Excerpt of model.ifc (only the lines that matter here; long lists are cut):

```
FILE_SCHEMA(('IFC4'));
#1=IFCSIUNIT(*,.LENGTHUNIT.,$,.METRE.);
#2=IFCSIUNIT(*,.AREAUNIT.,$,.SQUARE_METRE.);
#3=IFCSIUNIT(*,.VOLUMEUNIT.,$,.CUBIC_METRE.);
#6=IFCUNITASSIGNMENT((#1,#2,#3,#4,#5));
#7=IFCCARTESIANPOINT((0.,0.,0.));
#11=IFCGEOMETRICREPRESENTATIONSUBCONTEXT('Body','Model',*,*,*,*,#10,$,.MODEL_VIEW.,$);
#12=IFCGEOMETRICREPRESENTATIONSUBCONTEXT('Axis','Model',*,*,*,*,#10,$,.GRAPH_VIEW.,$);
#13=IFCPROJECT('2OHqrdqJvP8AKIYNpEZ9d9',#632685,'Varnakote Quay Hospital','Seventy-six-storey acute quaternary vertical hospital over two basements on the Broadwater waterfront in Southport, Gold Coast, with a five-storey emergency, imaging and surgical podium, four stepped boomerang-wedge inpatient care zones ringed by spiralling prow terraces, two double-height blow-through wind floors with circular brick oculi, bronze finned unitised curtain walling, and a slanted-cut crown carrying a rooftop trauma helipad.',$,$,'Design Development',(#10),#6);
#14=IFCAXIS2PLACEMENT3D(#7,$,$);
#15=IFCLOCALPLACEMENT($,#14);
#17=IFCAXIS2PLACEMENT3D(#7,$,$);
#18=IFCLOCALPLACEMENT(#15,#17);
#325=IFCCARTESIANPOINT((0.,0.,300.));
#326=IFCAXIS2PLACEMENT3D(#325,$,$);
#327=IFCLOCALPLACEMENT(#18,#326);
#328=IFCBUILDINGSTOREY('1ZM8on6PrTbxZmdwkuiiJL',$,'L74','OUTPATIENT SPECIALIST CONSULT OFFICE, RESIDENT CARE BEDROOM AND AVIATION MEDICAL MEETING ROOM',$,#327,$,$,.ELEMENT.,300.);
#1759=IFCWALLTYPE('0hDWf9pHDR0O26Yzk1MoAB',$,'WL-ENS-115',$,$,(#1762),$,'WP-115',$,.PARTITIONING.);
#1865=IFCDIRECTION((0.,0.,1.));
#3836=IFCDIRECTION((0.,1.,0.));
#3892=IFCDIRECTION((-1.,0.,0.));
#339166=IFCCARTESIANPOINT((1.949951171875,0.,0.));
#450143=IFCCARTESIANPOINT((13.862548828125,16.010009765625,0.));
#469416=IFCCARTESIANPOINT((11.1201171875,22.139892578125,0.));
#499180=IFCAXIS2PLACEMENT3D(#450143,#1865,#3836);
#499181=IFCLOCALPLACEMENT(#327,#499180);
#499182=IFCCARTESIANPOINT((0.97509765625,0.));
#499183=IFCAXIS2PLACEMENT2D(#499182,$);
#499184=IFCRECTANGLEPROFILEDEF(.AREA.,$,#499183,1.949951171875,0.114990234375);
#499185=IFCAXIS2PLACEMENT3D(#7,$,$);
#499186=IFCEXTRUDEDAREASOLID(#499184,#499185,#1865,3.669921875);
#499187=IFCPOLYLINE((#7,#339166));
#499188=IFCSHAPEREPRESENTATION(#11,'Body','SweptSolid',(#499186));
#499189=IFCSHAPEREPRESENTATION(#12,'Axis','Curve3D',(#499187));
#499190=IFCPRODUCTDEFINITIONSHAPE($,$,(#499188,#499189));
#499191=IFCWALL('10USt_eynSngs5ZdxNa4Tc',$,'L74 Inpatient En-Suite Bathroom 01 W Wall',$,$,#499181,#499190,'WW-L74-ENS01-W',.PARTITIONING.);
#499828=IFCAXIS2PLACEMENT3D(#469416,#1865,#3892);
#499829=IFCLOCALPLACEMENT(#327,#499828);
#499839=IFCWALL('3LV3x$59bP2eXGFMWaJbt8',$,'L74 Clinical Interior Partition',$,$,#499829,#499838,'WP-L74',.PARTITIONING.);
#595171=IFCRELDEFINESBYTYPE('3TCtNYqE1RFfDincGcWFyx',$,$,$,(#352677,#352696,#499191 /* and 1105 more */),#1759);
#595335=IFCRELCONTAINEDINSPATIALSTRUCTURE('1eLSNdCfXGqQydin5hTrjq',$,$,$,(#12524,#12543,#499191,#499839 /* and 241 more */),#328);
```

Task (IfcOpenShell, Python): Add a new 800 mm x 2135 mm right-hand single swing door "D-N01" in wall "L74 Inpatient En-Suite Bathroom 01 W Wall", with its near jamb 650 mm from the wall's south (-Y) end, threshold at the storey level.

```python
import numpy as np
import ifcopenshell
import ifcopenshell.api.feature
import ifcopenshell.api.geometry
import ifcopenshell.api.root
import ifcopenshell.api.spatial
import ifcopenshell.geom
import ifcopenshell.util.element
import ifcopenshell.util.placement
import ifcopenshell.util.representation
import ifcopenshell.util.shape
import ifcopenshell.util.unit

model = ifcopenshell.open("model.ifc")
unit_scale = ifcopenshell.util.unit.calculate_unit_scale(model)
settings = ifcopenshell.geom.settings()


def volume(element):
    """Net volume in cubic metres, openings subtracted."""
    shape = ifcopenshell.geom.create_shape(settings, element)
    return ifcopenshell.util.shape.get_volume(shape.geometry)


wall = model.by_guid("10USt_eynSngs5ZdxNa4Tc")
storey = ifcopenshell.util.element.get_container(wall, ifc_class="IfcBuildingStorey")
context = ifcopenshell.util.representation.get_context(model, "Model", "Body", "MODEL_VIEW")
before = volume(wall)

width, height, from_end, sill = 0.8, 2.135, 0.65, 0.0  # metres

# The wall runs along its own X axis, and the end named is its -X end.
wall_shape = ifcopenshell.geom.create_shape(settings, wall)
x, y, z = ifcopenshell.util.shape.get_vertices(wall_shape.geometry).T
start = x.min() + from_end
face, thickness = float(y.min()), float(y.max() - y.min())
wall_matrix = ifcopenshell.util.placement.get_local_placement(wall.ObjectPlacement)
level = ifcopenshell.util.placement.get_local_placement(storey.ObjectPlacement)[2, 3]


def in_wall(x, y):
    """Placement at x, y metres in the wall's axes, at sill height."""
    matrix = wall_matrix.copy()
    matrix[:, 3] = wall_matrix @ np.array([x / unit_scale, y / unit_scale, 0.0, 1.0])
    matrix[2, 3] = level + sill / unit_scale
    return matrix


# Opening: a box that overshoots both wall faces by 50 mm.
opening = ifcopenshell.api.root.create_entity(model, ifc_class="IfcOpeningElement", predefined_type="OPENING")
box = ifcopenshell.api.geometry.add_wall_representation(
    model, context=context, length=width, height=height, thickness=thickness + 0.1
)
ifcopenshell.api.geometry.assign_representation(model, product=opening, representation=box)
ifcopenshell.api.geometry.edit_object_placement(model, product=opening, matrix=in_wall(start, face - 0.05), is_si=False)
ifcopenshell.api.feature.add_feature(model, feature=opening, element=wall)

door = ifcopenshell.api.root.create_entity(model, ifc_class="IfcDoor", name="D-N01", predefined_type="DOOR")
door.OverallWidth, door.OverallHeight = width / unit_scale, height / unit_scale
door.OperationType = "SINGLE_SWING_RIGHT"
body = ifcopenshell.api.geometry.add_door_representation(
    model,
    context=context,
    overall_width=door.OverallWidth,
    overall_height=door.OverallHeight,
    operation_type="SINGLE_SWING_RIGHT",
    lining_properties={"LiningDepth": thickness / unit_scale, "ThresholdDepth": thickness / unit_scale},
)
ifcopenshell.api.geometry.assign_representation(model, product=door, representation=body)
ifcopenshell.api.spatial.assign_container(model, products=[door], relating_structure=storey)
ifcopenshell.api.feature.add_filling(model, opening=opening, element=door)

# The lining spans the wall, so the door starts at the wall face.
ifcopenshell.api.geometry.edit_object_placement(model, product=door, matrix=in_wall(start, face), is_si=False)

after = volume(wall)

print(f"wall volume {before:.3f} -> {after:.3f} m3")

model.write("model_updated.ifc")
```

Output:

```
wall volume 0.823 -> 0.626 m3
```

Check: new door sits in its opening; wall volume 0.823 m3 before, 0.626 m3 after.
